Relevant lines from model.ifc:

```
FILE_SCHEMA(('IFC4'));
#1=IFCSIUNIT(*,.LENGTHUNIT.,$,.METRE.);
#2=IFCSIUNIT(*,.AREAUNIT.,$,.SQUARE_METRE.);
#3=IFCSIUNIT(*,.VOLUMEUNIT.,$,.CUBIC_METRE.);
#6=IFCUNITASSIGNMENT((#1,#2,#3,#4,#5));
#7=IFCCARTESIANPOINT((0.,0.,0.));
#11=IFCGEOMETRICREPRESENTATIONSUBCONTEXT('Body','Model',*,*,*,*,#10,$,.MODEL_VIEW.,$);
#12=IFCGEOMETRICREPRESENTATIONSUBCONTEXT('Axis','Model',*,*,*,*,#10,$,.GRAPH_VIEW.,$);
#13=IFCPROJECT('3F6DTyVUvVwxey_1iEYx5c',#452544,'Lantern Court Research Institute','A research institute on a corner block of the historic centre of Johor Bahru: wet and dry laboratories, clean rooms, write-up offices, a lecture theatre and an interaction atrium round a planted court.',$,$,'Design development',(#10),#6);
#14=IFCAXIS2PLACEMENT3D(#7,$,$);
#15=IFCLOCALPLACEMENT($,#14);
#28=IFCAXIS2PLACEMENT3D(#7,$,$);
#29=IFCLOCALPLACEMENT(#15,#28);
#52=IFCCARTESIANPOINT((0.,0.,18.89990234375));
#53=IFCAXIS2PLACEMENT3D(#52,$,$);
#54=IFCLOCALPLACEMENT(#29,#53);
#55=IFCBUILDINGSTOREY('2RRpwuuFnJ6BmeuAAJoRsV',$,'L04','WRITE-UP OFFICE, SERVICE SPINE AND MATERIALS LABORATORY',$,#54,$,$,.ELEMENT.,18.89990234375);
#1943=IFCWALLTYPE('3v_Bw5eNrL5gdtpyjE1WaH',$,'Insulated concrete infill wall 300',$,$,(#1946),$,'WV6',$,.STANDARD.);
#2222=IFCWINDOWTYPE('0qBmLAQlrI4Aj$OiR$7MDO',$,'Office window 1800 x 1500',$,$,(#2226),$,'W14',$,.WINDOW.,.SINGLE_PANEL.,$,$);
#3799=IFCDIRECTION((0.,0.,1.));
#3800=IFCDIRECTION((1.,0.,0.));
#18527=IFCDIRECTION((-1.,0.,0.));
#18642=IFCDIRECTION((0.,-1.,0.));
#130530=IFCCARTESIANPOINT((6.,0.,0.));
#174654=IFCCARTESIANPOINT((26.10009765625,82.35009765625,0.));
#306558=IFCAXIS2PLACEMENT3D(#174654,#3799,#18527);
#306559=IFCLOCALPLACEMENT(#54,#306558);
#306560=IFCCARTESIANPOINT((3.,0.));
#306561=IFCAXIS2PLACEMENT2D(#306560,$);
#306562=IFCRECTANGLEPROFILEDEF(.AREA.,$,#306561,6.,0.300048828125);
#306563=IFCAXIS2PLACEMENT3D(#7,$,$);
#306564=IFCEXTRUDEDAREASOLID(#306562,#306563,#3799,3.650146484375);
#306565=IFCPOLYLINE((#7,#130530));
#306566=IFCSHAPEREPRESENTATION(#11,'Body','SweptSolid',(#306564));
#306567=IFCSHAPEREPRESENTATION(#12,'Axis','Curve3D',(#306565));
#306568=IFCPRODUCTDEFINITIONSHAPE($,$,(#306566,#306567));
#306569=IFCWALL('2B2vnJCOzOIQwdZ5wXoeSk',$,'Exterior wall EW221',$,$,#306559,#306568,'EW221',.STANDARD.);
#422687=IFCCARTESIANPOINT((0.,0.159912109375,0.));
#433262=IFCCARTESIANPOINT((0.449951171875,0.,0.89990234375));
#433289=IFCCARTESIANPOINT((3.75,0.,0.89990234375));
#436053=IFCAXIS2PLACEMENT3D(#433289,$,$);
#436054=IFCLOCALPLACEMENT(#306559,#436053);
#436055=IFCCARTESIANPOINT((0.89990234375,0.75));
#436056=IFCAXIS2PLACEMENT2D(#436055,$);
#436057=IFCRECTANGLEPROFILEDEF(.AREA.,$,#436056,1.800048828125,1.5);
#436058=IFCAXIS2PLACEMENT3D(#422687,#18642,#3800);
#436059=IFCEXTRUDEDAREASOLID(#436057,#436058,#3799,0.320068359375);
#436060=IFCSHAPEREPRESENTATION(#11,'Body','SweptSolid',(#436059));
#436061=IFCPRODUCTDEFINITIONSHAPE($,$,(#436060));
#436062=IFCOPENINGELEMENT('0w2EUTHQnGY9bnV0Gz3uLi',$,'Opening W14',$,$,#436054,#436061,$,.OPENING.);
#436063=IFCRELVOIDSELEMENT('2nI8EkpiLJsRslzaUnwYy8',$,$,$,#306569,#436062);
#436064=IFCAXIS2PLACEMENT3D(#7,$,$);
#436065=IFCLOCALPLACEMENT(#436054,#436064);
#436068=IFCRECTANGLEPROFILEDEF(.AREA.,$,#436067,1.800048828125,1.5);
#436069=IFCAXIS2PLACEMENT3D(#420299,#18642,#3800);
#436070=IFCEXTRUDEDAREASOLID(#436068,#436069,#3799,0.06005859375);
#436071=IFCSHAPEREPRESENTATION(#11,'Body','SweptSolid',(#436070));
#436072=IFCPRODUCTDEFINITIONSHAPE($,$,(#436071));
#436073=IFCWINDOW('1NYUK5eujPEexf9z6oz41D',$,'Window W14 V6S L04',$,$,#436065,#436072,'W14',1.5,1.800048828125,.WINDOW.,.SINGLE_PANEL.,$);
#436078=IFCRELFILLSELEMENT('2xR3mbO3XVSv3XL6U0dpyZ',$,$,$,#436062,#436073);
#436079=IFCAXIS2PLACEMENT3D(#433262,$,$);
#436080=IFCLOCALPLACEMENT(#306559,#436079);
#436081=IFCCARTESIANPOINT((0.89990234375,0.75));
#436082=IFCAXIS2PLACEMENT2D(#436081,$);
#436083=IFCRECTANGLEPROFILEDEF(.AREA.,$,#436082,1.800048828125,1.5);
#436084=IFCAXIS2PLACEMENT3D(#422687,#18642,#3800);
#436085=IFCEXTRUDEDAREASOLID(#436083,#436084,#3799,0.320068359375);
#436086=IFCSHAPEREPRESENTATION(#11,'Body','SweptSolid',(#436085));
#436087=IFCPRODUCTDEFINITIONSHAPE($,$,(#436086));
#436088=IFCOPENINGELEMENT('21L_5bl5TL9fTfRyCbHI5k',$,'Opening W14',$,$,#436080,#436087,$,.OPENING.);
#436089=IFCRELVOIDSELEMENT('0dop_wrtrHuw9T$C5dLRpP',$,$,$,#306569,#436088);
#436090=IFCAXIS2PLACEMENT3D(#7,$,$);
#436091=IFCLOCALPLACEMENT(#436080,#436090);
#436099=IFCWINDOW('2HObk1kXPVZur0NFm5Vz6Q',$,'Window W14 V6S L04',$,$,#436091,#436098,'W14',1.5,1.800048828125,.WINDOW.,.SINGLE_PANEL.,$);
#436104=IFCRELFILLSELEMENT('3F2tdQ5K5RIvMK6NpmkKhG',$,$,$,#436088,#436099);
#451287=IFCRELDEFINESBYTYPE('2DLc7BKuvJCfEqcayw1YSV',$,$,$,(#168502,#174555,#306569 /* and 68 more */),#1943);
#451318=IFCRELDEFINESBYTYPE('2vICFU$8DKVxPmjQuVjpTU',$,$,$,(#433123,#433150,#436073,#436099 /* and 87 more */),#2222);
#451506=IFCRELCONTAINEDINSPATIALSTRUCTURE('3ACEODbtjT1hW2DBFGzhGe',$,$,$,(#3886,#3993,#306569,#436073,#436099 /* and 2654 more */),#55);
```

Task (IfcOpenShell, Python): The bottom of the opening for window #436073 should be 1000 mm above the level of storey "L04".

```python
import numpy as np
import ifcopenshell
import ifcopenshell.api.geometry
import ifcopenshell.geom
import ifcopenshell.util.element
import ifcopenshell.util.placement
import ifcopenshell.util.shape
import ifcopenshell.util.unit

model = ifcopenshell.open("model.ifc")
unit_scale = ifcopenshell.util.unit.calculate_unit_scale(model)

window = model.by_id(436073)
opening = window.FillsVoids[0].RelatingOpeningElement
storey = ifcopenshell.util.element.get_container(window, ifc_class="IfcBuildingStorey")
level = ifcopenshell.util.placement.get_local_placement(storey.ObjectPlacement)[2, 3]

# The opening's origin need not be at the sill, so measure its lowest point.
shape = ifcopenshell.geom.create_shape(ifcopenshell.geom.settings(), opening)
bottom = ifcopenshell.util.shape.get_shape_bottom_elevation(shape, shape.geometry) / unit_scale
dz = level + 1 / unit_scale - bottom

shift = np.array([0.0, 0.0, dz])
# The window is placed relative to its opening, so it follows when the opening moves.
matrix = ifcopenshell.util.placement.get_local_placement(opening.ObjectPlacement)
matrix[:3, 3] += shift
ifcopenshell.api.geometry.edit_object_placement(
    model, product=opening, matrix=matrix, is_si=False, should_transform_children=True
)

print(f"moved by {dz * unit_scale:+.3f} m")

model.write("model_rev.ifc")
```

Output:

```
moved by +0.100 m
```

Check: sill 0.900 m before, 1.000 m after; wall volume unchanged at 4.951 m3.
